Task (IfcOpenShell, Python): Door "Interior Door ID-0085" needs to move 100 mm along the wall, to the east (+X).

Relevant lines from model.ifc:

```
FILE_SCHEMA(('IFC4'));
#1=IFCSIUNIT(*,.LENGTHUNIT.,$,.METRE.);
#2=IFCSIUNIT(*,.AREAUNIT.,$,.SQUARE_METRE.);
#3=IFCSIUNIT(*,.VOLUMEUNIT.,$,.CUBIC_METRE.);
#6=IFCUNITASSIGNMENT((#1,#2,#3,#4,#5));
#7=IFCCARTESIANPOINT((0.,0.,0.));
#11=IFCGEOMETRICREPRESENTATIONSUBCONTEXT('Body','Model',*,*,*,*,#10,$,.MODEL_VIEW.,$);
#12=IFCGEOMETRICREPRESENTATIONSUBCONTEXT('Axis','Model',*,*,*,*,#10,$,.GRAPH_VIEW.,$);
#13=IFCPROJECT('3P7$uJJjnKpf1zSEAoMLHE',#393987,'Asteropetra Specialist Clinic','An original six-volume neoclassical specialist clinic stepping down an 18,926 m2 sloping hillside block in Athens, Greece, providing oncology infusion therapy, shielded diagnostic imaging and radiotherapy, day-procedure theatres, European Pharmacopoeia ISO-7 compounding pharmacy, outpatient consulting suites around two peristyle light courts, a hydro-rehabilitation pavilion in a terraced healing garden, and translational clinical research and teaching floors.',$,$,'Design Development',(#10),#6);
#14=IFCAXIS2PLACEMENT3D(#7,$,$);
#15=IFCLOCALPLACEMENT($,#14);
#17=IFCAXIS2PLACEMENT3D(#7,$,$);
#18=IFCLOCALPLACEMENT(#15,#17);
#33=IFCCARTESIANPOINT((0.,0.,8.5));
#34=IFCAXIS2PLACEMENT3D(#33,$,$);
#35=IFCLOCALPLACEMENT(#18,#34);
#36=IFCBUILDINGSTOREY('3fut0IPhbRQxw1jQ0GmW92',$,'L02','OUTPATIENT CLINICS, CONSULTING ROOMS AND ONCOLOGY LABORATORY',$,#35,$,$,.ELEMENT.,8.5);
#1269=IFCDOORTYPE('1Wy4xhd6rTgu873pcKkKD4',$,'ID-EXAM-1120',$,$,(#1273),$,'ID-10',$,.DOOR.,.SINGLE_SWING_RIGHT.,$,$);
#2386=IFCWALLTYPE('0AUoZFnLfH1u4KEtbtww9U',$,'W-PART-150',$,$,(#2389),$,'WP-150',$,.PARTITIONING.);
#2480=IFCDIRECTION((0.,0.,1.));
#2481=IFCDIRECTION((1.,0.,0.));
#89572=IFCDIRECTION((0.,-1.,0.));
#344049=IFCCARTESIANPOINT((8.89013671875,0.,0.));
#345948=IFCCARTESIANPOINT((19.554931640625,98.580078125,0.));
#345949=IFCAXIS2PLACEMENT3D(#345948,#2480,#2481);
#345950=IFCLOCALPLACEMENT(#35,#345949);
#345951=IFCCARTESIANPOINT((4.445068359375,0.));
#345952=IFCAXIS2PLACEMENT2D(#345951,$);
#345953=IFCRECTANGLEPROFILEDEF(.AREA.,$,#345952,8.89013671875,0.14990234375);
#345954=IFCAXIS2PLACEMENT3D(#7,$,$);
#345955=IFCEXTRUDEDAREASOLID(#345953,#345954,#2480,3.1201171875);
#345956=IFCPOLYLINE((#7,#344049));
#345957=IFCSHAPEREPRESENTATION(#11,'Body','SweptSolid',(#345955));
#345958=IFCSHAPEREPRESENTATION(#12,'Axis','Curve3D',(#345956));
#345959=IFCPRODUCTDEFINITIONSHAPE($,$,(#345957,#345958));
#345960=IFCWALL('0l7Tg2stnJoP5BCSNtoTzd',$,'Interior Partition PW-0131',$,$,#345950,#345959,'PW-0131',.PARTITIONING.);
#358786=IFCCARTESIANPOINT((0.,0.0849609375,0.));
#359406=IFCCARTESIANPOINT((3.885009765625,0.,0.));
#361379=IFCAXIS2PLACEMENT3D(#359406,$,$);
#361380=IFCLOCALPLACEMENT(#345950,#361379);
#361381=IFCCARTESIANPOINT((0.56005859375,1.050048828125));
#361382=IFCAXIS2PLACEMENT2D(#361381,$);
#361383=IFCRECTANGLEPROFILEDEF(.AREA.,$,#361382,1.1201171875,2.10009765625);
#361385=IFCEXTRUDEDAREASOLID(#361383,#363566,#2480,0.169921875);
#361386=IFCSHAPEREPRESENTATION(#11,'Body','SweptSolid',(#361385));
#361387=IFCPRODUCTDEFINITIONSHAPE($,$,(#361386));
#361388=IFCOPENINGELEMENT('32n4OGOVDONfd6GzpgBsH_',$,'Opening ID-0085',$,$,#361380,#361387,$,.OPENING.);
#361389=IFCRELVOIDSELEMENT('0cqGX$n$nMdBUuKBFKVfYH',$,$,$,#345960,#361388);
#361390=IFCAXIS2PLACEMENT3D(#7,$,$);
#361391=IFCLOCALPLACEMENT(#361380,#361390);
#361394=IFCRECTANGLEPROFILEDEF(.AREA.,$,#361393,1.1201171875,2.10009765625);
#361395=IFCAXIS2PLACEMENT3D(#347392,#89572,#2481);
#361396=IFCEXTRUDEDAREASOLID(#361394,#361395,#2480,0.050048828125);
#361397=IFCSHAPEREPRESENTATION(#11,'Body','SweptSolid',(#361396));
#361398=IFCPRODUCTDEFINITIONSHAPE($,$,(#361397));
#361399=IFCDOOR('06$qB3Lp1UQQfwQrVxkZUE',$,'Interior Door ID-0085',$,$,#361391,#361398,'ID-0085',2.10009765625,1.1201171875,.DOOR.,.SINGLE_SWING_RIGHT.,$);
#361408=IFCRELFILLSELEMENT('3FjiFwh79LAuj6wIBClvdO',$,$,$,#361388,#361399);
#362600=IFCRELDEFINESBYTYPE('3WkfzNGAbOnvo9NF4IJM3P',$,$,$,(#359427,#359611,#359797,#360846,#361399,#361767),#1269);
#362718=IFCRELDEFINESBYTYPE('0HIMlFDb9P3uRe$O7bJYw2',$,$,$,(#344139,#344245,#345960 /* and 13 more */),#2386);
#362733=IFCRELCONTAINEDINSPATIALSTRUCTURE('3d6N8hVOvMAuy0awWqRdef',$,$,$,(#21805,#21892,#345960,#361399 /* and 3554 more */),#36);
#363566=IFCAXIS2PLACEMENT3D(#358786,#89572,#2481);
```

```python
import ifcopenshell
import ifcopenshell.api.geometry
import ifcopenshell.util.placement
import ifcopenshell.util.unit

model = ifcopenshell.open("model.ifc")
unit_scale = ifcopenshell.util.unit.calculate_unit_scale(model)

door = model.by_guid("06$qB3Lp1UQQfwQrVxkZUE")
opening = door.FillsVoids[0].RelatingOpeningElement
wall = opening.VoidsElements[0].RelatingBuildingElement

wall_matrix = ifcopenshell.util.placement.get_local_placement(wall.ObjectPlacement)
shift = wall_matrix[:3, 0] * 0.1 / unit_scale
before = ifcopenshell.util.placement.get_local_placement(door.ObjectPlacement)[:3, 3].copy()

# The door is placed relative to its opening, so it follows when the opening moves.
matrix = ifcopenshell.util.placement.get_local_placement(opening.ObjectPlacement)
matrix[:3, 3] += shift
ifcopenshell.api.geometry.edit_object_placement(
    model, product=opening, matrix=matrix, is_si=False, should_transform_children=True
)

after = ifcopenshell.util.placement.get_local_placement(door.ObjectPlacement)[:3, 3]
print("door moved by", (after - before).round(3) + 0.0)

model.write("model_rev.ifc")
```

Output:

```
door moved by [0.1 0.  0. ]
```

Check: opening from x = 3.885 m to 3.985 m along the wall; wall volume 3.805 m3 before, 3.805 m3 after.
